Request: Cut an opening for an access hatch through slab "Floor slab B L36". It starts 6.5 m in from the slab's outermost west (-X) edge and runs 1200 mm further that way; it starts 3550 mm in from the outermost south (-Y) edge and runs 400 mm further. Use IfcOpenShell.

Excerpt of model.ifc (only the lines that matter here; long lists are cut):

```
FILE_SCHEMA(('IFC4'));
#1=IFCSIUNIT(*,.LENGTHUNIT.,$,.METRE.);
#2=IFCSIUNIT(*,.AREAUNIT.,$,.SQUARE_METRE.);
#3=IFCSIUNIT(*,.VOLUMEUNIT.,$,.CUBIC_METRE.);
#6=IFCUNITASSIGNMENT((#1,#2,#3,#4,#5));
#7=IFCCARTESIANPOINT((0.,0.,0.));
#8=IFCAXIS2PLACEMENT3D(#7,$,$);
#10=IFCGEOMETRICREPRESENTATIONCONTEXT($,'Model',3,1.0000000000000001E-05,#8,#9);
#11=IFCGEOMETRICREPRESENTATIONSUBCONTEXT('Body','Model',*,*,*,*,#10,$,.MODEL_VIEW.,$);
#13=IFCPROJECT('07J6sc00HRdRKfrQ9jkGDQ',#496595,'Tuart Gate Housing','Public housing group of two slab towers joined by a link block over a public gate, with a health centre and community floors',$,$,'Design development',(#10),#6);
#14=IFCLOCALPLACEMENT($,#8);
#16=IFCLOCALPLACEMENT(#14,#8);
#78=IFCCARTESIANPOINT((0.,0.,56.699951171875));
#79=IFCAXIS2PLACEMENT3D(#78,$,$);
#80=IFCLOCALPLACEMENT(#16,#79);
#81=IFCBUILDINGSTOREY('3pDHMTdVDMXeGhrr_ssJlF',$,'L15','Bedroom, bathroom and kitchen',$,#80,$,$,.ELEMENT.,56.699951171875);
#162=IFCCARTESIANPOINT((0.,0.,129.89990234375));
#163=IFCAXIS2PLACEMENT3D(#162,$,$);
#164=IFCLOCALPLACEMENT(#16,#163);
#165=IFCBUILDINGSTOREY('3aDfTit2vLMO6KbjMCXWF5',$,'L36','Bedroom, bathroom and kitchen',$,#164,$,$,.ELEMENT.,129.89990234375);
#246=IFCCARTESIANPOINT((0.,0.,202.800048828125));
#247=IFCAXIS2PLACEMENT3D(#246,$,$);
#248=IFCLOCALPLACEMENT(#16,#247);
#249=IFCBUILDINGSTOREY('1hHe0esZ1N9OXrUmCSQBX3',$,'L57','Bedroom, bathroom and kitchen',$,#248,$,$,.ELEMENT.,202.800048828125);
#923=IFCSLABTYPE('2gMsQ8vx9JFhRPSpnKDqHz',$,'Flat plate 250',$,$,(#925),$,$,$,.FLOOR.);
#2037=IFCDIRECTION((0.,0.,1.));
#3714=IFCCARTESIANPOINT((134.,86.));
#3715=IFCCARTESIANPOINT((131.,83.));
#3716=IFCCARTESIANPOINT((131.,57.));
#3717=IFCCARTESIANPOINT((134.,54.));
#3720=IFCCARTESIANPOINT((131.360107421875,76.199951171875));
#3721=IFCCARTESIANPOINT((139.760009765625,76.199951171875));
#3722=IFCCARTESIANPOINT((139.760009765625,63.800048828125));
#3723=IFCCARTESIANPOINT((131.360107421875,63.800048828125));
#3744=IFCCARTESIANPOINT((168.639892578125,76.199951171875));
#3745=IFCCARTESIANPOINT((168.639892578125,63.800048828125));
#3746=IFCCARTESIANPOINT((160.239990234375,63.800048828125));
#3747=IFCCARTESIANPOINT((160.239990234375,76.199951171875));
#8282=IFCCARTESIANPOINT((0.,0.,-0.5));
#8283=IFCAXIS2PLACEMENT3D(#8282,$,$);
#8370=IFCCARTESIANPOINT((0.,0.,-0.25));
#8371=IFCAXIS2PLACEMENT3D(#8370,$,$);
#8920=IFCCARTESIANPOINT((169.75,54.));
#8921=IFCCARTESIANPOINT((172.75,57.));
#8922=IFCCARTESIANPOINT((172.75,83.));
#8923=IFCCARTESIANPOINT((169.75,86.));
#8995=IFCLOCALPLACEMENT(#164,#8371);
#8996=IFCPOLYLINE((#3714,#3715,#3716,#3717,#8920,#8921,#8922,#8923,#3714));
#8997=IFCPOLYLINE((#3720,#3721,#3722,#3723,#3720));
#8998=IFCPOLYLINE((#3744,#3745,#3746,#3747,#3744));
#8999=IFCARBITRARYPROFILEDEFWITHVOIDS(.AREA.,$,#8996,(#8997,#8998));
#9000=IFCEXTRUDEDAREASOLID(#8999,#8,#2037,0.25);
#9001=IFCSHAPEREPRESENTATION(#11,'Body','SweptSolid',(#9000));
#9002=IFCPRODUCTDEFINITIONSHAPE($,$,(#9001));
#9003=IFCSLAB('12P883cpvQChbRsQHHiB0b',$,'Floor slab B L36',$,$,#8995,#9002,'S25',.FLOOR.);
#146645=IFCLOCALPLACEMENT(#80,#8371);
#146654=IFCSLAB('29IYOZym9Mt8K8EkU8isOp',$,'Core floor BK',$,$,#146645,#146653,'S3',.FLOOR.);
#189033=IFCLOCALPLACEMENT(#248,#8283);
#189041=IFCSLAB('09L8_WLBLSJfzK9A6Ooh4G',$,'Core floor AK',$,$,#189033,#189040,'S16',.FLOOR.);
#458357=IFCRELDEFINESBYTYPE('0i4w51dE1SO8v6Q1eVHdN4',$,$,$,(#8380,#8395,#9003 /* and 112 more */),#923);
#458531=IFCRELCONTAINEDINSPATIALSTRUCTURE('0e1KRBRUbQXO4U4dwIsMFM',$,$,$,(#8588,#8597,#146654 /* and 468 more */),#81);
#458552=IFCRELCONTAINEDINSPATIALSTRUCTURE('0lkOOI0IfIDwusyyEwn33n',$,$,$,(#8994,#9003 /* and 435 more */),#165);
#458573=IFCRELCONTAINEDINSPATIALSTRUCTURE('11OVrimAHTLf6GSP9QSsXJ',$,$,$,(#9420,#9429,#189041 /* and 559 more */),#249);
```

```python
import numpy as np
import ifcopenshell
import ifcopenshell.api.feature
import ifcopenshell.api.geometry
import ifcopenshell.api.root
import ifcopenshell.geom
import ifcopenshell.util.placement
import ifcopenshell.util.representation
import ifcopenshell.util.shape
import ifcopenshell.util.unit

model = ifcopenshell.open("model.ifc")
unit_scale = ifcopenshell.util.unit.calculate_unit_scale(model)
settings = ifcopenshell.geom.settings()


def volume(element):
    """Net volume in cubic metres, openings subtracted."""
    shape = ifcopenshell.geom.create_shape(settings, element)
    return ifcopenshell.util.shape.get_volume(shape.geometry)


slab = model.by_id(9003)
before = volume(slab)

# Extent in the slab's own axes, in metres. The edges named are its -X and -Y sides.
slab_shape = ifcopenshell.geom.create_shape(settings, slab)
vertices = ifcopenshell.util.shape.get_vertices(slab_shape.geometry)
x_min, y_min, bottom = vertices.min(axis=0)
top = vertices[:, 2].max()

opening = ifcopenshell.api.root.create_entity(model, ifc_class="IfcOpeningElement", name="Access hatch opening", predefined_type="OPENING")
context = ifcopenshell.util.representation.get_context(model, "Model", "Body", "MODEL_VIEW")
width, depth = 1.2, 0.4
outline = [(0.0, 0.0), (width, 0.0), (width, depth), (0.0, depth), (0.0, 0.0)]
# Overshoot both faces by 50 mm so the cut is clean.
shape = ifcopenshell.api.geometry.add_slab_representation(
    model, context=context, depth=top - bottom + 0.1, polyline=outline
)
ifcopenshell.api.geometry.assign_representation(model, product=opening, representation=shape)

matrix = ifcopenshell.util.placement.get_local_placement(slab.ObjectPlacement)
matrix[:, 3] = matrix @ np.append(np.array([x_min + 6.5, y_min + 3.55, bottom - 0.05]) / unit_scale, 1.0)
ifcopenshell.api.geometry.edit_object_placement(model, product=opening, matrix=matrix, is_si=False)
ifcopenshell.api.feature.add_feature(model, feature=opening, element=slab)

after = volume(slab)

print(f"slab volume {before:.3f} -> {after:.3f} m3")

model.write("model-out.ifc")
```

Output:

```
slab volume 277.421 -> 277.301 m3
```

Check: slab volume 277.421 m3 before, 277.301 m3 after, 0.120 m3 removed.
